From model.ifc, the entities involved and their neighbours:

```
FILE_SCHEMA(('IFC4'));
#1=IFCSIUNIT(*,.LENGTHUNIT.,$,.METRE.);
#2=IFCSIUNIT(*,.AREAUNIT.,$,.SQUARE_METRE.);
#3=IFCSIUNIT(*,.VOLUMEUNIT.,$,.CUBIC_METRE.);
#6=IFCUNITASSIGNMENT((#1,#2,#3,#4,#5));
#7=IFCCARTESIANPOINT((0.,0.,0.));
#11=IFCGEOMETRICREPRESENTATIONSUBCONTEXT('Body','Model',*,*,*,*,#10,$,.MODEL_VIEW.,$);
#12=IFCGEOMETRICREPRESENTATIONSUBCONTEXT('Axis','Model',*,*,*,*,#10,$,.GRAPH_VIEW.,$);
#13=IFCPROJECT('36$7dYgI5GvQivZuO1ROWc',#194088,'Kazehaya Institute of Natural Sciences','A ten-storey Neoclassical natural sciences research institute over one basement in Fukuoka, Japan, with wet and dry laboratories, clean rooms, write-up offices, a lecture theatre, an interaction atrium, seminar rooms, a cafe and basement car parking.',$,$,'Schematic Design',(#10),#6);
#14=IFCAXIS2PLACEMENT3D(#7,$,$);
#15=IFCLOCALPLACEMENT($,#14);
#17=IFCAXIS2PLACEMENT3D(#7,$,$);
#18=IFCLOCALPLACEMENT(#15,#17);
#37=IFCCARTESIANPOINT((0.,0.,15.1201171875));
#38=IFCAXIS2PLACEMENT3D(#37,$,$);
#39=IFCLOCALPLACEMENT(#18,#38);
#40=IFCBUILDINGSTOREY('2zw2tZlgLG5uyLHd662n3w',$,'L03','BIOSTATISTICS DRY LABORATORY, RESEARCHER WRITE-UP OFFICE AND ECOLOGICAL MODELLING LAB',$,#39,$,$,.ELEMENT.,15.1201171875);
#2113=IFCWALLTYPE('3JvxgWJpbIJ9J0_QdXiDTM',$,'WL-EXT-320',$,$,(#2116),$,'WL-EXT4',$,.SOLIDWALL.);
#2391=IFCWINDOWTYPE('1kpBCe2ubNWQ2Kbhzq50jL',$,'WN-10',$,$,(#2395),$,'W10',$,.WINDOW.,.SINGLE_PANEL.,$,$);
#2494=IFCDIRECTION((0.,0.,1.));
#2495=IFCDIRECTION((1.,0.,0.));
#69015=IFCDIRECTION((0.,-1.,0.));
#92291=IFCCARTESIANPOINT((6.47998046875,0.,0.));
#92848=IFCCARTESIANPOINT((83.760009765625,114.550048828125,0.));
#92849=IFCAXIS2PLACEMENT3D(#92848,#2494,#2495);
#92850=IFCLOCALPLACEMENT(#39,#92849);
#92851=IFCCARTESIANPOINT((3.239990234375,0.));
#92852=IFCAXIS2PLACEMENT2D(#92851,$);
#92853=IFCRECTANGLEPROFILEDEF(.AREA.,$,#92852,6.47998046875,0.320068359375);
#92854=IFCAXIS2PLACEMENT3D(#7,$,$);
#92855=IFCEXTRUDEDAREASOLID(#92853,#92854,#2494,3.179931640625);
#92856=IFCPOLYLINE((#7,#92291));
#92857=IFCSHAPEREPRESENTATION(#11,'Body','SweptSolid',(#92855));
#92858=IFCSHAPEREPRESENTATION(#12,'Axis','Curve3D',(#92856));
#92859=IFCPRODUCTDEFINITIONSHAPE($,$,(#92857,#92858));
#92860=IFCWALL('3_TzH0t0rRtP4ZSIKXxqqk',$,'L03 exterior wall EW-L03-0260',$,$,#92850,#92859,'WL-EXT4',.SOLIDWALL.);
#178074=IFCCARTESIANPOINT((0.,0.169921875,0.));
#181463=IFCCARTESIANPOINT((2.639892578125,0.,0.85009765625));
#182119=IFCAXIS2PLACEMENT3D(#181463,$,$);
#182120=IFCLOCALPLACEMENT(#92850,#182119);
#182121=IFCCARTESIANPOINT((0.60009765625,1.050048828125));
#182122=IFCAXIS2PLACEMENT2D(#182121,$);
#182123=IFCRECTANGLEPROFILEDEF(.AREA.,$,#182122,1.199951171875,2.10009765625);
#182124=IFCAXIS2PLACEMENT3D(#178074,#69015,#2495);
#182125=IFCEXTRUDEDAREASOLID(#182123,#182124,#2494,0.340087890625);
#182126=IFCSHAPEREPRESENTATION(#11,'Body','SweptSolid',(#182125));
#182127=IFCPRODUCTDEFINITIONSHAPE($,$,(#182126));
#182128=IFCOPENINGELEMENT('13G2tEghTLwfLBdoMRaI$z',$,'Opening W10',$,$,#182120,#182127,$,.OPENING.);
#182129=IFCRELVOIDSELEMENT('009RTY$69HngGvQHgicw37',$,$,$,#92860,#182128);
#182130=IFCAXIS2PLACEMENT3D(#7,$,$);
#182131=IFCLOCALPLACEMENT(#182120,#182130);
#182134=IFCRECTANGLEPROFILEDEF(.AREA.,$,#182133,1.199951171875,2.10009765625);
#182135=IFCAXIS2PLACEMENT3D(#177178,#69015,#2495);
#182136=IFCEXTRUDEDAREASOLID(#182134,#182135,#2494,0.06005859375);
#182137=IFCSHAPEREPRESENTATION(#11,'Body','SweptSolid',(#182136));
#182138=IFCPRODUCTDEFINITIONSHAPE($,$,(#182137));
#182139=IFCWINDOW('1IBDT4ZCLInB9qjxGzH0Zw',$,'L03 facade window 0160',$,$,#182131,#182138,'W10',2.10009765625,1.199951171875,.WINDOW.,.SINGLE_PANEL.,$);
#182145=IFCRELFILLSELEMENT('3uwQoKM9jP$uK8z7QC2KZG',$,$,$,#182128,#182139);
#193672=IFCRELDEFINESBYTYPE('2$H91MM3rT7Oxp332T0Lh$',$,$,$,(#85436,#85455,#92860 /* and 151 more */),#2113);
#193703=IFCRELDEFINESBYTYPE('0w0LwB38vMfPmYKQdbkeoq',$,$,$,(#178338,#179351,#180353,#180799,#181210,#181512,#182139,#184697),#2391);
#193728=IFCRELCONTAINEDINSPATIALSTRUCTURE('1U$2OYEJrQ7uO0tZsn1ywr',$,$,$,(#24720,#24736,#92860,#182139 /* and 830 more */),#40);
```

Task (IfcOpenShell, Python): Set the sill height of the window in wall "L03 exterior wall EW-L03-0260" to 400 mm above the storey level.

```python
import numpy as np
import ifcopenshell
import ifcopenshell.api.geometry
import ifcopenshell.geom
import ifcopenshell.util.element
import ifcopenshell.util.placement
import ifcopenshell.util.shape
import ifcopenshell.util.unit

model = ifcopenshell.open("model.ifc")
unit_scale = ifcopenshell.util.unit.calculate_unit_scale(model)

window = model.by_guid("1IBDT4ZCLInB9qjxGzH0Zw")
opening = window.FillsVoids[0].RelatingOpeningElement
storey = ifcopenshell.util.element.get_container(window, ifc_class="IfcBuildingStorey")
level = ifcopenshell.util.placement.get_local_placement(storey.ObjectPlacement)[2, 3]

# The opening's origin need not be at the sill, so measure its lowest point.
shape = ifcopenshell.geom.create_shape(ifcopenshell.geom.settings(), opening)
bottom = ifcopenshell.util.shape.get_shape_bottom_elevation(shape, shape.geometry) / unit_scale
dz = level + 0.4 / unit_scale - bottom

shift = np.array([0.0, 0.0, dz])
# The window is placed relative to its opening, so it follows when the opening moves.
matrix = ifcopenshell.util.placement.get_local_placement(opening.ObjectPlacement)
matrix[:3, 3] += shift
ifcopenshell.api.geometry.edit_object_placement(
    model, product=opening, matrix=matrix, is_si=False, should_transform_children=True
)

print(f"moved by {dz * unit_scale:+.3f} m")

model.write("model-out.ifc")
```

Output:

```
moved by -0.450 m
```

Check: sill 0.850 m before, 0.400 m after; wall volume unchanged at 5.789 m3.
